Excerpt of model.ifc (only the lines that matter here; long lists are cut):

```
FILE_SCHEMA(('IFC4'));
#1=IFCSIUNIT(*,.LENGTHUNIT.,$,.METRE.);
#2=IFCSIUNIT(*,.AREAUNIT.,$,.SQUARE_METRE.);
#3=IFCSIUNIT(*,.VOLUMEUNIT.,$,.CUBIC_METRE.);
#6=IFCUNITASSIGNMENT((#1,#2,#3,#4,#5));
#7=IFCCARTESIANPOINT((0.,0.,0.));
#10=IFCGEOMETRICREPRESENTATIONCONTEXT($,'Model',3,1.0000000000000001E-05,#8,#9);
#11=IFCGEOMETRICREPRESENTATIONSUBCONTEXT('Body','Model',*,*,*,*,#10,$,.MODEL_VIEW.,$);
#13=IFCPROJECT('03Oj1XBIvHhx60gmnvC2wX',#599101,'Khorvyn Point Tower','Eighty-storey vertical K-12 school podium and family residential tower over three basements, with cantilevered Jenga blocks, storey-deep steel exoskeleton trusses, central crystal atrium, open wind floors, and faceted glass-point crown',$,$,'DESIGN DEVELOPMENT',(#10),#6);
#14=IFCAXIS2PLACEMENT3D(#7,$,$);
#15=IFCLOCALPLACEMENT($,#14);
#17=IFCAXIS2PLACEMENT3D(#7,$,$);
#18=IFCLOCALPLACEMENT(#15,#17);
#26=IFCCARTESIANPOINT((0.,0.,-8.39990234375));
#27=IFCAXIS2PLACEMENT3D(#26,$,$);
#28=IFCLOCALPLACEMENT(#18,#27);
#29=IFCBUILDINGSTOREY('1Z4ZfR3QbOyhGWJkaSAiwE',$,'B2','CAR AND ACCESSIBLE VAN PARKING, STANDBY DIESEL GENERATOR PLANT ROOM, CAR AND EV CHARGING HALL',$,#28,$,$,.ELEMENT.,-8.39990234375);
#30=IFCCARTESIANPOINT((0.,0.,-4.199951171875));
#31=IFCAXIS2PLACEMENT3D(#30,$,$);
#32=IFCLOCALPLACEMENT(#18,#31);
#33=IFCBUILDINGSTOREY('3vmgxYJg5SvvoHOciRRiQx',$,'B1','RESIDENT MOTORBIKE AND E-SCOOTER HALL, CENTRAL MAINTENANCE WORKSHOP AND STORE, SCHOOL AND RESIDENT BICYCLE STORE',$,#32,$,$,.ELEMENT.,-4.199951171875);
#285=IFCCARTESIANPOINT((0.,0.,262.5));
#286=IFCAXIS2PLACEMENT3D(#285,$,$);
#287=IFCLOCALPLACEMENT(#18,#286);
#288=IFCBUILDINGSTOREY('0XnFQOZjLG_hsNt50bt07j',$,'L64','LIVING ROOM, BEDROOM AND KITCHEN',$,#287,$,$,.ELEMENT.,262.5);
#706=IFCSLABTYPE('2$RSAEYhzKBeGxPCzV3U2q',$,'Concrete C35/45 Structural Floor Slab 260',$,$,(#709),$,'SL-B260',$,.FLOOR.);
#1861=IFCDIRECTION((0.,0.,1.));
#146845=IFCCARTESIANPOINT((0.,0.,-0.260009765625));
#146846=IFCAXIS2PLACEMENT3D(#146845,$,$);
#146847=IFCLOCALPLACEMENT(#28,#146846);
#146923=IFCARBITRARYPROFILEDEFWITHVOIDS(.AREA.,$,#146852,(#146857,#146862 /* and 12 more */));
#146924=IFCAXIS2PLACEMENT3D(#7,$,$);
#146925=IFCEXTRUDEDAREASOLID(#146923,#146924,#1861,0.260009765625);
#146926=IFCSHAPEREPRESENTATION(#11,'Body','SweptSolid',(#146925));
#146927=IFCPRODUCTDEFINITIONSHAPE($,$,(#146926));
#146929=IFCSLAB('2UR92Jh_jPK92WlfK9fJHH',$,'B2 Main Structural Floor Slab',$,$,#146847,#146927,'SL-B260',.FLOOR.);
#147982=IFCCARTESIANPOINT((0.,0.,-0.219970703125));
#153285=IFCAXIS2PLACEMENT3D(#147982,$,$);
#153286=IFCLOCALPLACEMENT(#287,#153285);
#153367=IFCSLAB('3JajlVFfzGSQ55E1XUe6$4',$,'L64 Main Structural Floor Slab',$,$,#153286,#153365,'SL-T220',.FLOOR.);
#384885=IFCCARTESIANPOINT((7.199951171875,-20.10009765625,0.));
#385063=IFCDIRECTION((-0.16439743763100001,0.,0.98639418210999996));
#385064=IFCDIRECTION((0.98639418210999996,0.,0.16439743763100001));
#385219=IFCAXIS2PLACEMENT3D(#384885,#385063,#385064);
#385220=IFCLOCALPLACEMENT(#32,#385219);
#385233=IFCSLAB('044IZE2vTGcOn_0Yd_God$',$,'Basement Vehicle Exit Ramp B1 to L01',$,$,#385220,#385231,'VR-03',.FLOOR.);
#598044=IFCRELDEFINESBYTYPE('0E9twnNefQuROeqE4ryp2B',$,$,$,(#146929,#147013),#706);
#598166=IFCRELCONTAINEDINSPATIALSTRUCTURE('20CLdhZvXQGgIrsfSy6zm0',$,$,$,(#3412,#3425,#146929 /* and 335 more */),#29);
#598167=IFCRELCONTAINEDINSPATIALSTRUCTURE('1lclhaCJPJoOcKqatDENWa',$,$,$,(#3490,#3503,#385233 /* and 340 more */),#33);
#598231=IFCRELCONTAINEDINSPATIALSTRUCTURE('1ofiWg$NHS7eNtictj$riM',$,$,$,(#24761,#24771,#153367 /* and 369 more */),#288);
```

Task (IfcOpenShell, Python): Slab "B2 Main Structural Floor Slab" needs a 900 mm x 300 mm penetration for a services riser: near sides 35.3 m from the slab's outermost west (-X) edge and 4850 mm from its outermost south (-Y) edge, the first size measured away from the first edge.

```python
import numpy as np
import ifcopenshell
import ifcopenshell.api.feature
import ifcopenshell.api.geometry
import ifcopenshell.api.root
import ifcopenshell.geom
import ifcopenshell.util.placement
import ifcopenshell.util.representation
import ifcopenshell.util.shape
import ifcopenshell.util.unit

model = ifcopenshell.open("model.ifc")
unit_scale = ifcopenshell.util.unit.calculate_unit_scale(model)
settings = ifcopenshell.geom.settings()


def volume(element):
    """Net volume in cubic metres, openings subtracted."""
    shape = ifcopenshell.geom.create_shape(settings, element)
    return ifcopenshell.util.shape.get_volume(shape.geometry)


slab = model.by_id(146929)
before = volume(slab)

# Extent in the slab's own axes, in metres. The edges named are its -X and -Y sides.
slab_shape = ifcopenshell.geom.create_shape(settings, slab)
vertices = ifcopenshell.util.shape.get_vertices(slab_shape.geometry)
x_min, y_min, bottom = vertices.min(axis=0)
top = vertices[:, 2].max()

opening = ifcopenshell.api.root.create_entity(model, ifc_class="IfcOpeningElement", name="Services riser opening", predefined_type="OPENING")
context = ifcopenshell.util.representation.get_context(model, "Model", "Body", "MODEL_VIEW")
width, depth = 0.9, 0.3
outline = [(0.0, 0.0), (width, 0.0), (width, depth), (0.0, depth), (0.0, 0.0)]
# Overshoot both faces by 50 mm so the cut is clean.
shape = ifcopenshell.api.geometry.add_slab_representation(
    model, context=context, depth=top - bottom + 0.1, polyline=outline
)
ifcopenshell.api.geometry.assign_representation(model, product=opening, representation=shape)

matrix = ifcopenshell.util.placement.get_local_placement(slab.ObjectPlacement)
matrix[:, 3] = matrix @ np.append(np.array([x_min + 35.3, y_min + 4.85, bottom - 0.05]) / unit_scale, 1.0)
ifcopenshell.api.geometry.edit_object_placement(model, product=opening, matrix=matrix, is_si=False)
ifcopenshell.api.feature.add_feature(model, feature=opening, element=slab)

after = volume(slab)

print(f"slab volume {before:.3f} -> {after:.3f} m3")

model.write("model_updated.ifc")
```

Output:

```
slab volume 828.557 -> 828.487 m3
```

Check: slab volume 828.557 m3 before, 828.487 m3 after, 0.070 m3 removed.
